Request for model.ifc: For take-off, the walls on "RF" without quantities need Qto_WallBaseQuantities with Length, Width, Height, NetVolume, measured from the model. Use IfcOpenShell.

First a look at what the model holds.

```python
import ifcopenshell
import ifcopenshell.util.element
import ifcopenshell.util.unit

model = ifcopenshell.open("model.ifc")
print(model.schema)
for unit_type in ("LENGTHUNIT", "AREAUNIT", "VOLUMEUNIT"):
    print(unit_type, ifcopenshell.util.unit.calculate_unit_scale(model, unit_type))
storey = next(s for s in model.by_type("IfcBuildingStorey") if s.Name == "RF")
walls = [e for e in ifcopenshell.util.element.get_decomposition(storey) if e.is_a("IfcWall")]
for e in sorted(walls, key=lambda e: e.id()):
    print(e.id(), e.is_a(), e.Name, list(ifcopenshell.util.element.get_psets(e, qtos_only=True)), sep=" | ")
```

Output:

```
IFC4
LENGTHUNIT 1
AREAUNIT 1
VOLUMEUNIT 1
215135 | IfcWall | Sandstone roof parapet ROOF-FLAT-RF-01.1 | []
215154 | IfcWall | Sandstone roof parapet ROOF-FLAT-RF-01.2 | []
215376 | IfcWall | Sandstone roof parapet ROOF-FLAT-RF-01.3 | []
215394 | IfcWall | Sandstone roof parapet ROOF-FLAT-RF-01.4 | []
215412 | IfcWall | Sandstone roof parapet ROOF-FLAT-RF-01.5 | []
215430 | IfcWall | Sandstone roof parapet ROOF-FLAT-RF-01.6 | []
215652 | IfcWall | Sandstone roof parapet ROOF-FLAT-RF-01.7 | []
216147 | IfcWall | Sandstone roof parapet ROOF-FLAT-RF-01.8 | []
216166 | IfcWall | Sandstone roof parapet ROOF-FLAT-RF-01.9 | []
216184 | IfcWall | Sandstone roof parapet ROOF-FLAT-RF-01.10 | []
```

```python
import ifcopenshell
import ifcopenshell.api.pset
import ifcopenshell.geom
import ifcopenshell.util.element
import ifcopenshell.util.shape
import ifcopenshell.util.unit

model = ifcopenshell.open("model.ifc")
unit_scale = ifcopenshell.util.unit.calculate_unit_scale(model)
volume_scale = ifcopenshell.util.unit.calculate_unit_scale(model, "VOLUMEUNIT")
settings = ifcopenshell.geom.settings()

storey = next(s for s in model.by_type("IfcBuildingStorey") if s.Name == "RF")
walls = [e for e in ifcopenshell.util.element.get_decomposition(storey) if e.is_a("IfcWall")]

for e in sorted(walls, key=lambda e: e.id()):
    if ifcopenshell.util.element.get_psets(e, qtos_only=True, should_inherit=False):
        continue
    # Geometry comes back in metres, in the element's own axes.
    shape = ifcopenshell.geom.create_shape(settings, e)
    values = {
        "Length": ifcopenshell.util.shape.get_x(shape.geometry) / unit_scale,
        "Width": ifcopenshell.util.shape.get_y(shape.geometry) / unit_scale,
        "Height": ifcopenshell.util.shape.get_z(shape.geometry) / unit_scale,
        "NetVolume": ifcopenshell.util.shape.get_volume(shape.geometry) / volume_scale,
    }
    qto = ifcopenshell.api.pset.add_qto(model, product=e, name="Qto_WallBaseQuantities")
    ifcopenshell.api.pset.edit_qto(model, qto=qto, properties=values)
    print(e.id(), {k: round(v, 3) for k, v in values.items()})

model.write("model_rev.ifc")
```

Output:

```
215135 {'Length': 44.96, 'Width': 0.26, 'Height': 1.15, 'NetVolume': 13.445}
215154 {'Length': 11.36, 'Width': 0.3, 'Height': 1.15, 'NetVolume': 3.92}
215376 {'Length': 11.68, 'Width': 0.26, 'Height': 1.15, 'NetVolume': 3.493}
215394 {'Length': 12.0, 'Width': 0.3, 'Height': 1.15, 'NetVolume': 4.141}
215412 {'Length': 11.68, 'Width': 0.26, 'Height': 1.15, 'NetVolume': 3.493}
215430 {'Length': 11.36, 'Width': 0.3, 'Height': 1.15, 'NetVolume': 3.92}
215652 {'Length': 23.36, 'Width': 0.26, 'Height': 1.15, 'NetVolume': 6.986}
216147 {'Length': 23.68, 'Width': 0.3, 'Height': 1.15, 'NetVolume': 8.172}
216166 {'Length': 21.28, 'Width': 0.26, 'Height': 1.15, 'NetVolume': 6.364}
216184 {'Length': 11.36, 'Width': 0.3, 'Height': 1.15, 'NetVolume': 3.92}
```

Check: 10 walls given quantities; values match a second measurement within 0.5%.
